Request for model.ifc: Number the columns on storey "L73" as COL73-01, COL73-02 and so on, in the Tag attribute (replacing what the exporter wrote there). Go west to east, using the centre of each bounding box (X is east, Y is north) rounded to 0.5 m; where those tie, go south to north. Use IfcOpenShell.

First a look at what the model holds.

```python
import ifcopenshell
import ifcopenshell.util.element
import ifcopenshell.util.placement

model = ifcopenshell.open("model.ifc")
print(model.schema)
storey = next(s for s in model.by_type("IfcBuildingStorey") if s.Name == "L73")
columns = [e for e in ifcopenshell.util.element.get_decomposition(storey) if e.is_a("IfcColumn")]
for e in sorted(columns, key=lambda e: e.id()):
    origin = ifcopenshell.util.placement.get_local_placement(e.ObjectPlacement)[:3, 3]
    print(e.id(), e.Tag, e.Name, origin.round(2) + 0.0, sep=" | ")
```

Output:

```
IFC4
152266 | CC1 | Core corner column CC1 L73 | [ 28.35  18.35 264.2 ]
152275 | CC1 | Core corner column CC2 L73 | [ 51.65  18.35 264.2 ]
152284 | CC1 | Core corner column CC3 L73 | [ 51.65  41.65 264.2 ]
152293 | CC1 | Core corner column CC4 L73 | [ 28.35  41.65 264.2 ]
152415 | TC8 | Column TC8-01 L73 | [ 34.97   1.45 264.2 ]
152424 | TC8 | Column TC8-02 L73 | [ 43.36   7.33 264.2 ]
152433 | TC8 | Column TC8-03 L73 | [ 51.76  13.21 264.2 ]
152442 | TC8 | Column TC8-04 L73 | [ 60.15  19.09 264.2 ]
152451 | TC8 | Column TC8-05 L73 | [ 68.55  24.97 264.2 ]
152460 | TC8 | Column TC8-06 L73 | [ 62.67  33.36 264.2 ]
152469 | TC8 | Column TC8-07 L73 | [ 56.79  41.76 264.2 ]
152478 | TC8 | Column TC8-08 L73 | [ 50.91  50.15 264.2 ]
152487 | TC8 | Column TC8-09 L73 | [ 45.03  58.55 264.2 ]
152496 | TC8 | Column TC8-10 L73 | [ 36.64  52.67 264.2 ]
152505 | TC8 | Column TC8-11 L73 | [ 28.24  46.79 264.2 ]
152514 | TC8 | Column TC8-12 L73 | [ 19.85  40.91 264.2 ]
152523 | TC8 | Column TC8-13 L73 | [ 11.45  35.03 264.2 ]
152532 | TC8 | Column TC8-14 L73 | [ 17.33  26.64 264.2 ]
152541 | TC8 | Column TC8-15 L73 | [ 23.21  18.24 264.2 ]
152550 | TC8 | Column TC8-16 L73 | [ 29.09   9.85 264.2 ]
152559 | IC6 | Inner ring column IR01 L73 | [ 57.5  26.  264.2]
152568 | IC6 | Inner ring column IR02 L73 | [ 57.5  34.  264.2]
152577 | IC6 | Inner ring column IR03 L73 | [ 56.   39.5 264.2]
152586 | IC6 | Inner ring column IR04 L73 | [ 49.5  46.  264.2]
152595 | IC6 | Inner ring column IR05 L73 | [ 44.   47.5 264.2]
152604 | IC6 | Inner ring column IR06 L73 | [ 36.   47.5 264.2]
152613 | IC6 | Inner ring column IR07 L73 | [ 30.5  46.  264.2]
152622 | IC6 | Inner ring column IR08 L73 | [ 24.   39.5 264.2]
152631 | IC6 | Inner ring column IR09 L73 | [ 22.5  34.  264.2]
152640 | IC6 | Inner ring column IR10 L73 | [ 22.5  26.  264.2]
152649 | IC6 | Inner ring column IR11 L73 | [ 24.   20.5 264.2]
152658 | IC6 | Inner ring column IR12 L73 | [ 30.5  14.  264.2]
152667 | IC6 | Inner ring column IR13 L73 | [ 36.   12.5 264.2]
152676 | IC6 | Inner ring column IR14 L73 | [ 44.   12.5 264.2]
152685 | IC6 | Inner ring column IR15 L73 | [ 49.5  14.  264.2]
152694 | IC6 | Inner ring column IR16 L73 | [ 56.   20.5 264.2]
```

```python
import ifcopenshell
import ifcopenshell.geom
import ifcopenshell.util.element
import ifcopenshell.util.shape

model = ifcopenshell.open("model.ifc")
settings = ifcopenshell.geom.settings()
settings.set("use-world-coords", True)


def centre(element):
    shape = ifcopenshell.geom.create_shape(settings, element)
    return ifcopenshell.util.shape.get_bbox_centroid(shape.geometry)


storey = next(s for s in model.by_type("IfcBuildingStorey") if s.Name == "L73")
columns = [e for e in ifcopenshell.util.element.get_decomposition(storey) if e.is_a("IfcColumn")]

# Insertion points can sit at a corner or the storey origin, so sort by the geometry (in metres).
centres = {e: centre(e) for e in columns}
columns.sort(key=lambda e: (round(centres[e][0] / 0.5), centres[e][1]))

for i, e in enumerate(columns, start=1):
    number = f"COL73-{i:02d}"
    e.Tag = number
    print(e.id(), number)

model.write("model_updated.ifc")
```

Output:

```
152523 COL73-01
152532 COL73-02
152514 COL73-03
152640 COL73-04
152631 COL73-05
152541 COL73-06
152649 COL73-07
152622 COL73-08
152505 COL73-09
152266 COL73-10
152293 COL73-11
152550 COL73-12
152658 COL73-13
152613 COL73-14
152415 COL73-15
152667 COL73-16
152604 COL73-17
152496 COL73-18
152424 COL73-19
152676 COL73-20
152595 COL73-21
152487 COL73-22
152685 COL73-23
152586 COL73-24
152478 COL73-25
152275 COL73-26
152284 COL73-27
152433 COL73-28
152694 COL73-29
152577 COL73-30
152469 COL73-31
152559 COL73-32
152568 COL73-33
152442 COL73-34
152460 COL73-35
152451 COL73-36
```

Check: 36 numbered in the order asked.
